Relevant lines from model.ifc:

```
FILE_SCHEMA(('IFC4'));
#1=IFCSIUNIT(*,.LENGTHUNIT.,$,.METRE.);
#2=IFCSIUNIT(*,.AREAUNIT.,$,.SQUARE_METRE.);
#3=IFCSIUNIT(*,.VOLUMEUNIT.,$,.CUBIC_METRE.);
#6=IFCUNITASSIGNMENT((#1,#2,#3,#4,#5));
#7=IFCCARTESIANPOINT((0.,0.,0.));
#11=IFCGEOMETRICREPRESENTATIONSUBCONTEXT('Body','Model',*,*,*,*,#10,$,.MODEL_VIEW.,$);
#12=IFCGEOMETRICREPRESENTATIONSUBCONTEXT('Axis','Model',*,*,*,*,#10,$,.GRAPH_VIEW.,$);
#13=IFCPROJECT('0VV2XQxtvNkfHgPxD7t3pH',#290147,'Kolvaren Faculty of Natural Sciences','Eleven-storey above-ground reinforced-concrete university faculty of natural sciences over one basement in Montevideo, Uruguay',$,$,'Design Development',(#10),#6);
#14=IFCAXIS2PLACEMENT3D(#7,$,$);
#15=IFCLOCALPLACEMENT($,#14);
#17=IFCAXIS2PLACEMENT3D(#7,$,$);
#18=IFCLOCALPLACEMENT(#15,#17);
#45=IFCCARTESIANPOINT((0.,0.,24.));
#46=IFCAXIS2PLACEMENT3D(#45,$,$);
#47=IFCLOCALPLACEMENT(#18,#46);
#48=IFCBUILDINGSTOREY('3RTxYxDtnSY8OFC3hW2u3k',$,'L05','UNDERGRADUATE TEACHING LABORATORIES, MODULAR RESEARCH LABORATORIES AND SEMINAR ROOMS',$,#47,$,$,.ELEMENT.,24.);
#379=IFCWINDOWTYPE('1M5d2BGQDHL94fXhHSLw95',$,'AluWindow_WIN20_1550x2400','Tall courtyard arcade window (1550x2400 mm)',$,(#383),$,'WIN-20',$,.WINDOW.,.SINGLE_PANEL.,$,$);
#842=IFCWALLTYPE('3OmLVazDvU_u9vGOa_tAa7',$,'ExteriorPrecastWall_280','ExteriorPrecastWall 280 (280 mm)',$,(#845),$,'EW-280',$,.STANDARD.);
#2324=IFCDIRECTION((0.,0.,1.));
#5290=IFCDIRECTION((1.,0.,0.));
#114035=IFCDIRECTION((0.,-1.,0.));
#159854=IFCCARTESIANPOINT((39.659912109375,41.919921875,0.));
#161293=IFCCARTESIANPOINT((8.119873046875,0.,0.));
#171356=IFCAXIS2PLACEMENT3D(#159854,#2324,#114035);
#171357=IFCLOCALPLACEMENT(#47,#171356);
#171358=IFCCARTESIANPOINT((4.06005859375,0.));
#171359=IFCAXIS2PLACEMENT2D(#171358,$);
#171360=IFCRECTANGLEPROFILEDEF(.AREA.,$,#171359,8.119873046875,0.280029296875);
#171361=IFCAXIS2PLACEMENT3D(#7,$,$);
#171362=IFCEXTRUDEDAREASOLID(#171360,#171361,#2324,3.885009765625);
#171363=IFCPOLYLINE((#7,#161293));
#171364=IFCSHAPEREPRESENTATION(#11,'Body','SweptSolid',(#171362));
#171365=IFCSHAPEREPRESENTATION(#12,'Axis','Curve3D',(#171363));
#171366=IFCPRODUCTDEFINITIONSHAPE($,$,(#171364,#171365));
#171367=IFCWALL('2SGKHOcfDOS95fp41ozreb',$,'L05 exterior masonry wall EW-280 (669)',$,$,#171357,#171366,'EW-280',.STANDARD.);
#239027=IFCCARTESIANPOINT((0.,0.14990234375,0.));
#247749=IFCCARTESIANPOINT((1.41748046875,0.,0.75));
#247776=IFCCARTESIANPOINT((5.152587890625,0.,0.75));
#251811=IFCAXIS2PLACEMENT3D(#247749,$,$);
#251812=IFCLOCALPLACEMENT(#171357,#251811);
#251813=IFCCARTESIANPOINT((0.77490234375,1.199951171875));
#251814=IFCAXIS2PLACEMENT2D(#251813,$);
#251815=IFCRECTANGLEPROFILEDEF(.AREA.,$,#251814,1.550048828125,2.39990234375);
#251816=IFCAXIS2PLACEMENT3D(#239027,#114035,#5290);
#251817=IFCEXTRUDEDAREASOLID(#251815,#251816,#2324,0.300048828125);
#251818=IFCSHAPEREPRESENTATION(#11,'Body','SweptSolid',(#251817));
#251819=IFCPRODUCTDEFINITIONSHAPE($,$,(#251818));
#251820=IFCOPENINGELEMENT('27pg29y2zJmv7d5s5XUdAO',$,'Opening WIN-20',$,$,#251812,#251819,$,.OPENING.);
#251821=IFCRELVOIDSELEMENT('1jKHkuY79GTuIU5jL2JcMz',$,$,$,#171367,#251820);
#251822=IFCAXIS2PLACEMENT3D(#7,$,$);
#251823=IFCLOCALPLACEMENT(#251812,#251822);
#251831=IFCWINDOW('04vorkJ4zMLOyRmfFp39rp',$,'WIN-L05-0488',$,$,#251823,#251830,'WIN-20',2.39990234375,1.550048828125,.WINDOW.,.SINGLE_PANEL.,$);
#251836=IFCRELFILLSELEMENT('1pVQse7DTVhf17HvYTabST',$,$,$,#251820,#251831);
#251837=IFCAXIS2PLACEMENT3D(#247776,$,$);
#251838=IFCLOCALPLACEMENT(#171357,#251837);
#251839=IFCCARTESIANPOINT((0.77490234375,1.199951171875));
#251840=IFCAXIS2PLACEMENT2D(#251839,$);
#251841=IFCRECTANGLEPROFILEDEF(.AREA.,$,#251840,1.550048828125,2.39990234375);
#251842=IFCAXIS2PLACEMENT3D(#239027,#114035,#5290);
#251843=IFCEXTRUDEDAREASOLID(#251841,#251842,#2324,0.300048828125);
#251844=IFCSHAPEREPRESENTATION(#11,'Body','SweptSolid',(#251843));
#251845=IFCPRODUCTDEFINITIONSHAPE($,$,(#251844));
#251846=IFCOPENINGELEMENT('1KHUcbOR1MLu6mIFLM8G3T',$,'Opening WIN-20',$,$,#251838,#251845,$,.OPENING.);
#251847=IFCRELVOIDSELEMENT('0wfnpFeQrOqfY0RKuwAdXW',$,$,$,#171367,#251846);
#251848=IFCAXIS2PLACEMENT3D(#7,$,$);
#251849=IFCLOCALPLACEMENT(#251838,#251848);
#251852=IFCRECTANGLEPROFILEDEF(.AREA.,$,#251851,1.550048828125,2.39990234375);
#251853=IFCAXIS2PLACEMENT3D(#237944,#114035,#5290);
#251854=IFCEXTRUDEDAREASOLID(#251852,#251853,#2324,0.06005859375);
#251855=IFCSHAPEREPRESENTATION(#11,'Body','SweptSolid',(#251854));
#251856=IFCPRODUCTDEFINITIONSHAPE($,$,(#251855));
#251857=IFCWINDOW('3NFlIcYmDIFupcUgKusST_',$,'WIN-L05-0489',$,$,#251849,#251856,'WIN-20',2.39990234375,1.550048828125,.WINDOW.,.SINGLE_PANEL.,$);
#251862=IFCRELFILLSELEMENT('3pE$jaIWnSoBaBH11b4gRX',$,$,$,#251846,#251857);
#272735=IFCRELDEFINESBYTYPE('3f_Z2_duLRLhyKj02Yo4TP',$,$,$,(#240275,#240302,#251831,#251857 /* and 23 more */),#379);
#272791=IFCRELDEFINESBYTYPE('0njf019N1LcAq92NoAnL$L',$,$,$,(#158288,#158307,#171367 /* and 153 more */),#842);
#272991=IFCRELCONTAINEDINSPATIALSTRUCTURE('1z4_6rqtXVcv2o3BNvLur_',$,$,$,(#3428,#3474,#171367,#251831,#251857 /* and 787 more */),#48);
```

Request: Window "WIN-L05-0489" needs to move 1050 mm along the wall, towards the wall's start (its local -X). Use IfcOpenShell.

```python
import ifcopenshell
import ifcopenshell.api.geometry
import ifcopenshell.util.placement

model = ifcopenshell.open("model.ifc")

window = model.by_guid("3NFlIcYmDIFupcUgKusST_")
opening = window.FillsVoids[0].RelatingOpeningElement
wall = opening.VoidsElements[0].RelatingBuildingElement

wall_matrix = ifcopenshell.util.placement.get_local_placement(wall.ObjectPlacement)
shift = wall_matrix[:3, 0] * -1.05
before = ifcopenshell.util.placement.get_local_placement(window.ObjectPlacement)[:3, 3].copy()

# The window is placed relative to its opening, so it follows when the opening moves.
matrix = ifcopenshell.util.placement.get_local_placement(opening.ObjectPlacement)
matrix[:3, 3] += shift
ifcopenshell.api.geometry.edit_object_placement(
    model, product=opening, matrix=matrix, is_si=False, should_transform_children=True
)

after = ifcopenshell.util.placement.get_local_placement(window.ObjectPlacement)[:3, 3]
print("window moved by", (after - before).round(3) + 0.0)

model.write("model_v2.ifc")
```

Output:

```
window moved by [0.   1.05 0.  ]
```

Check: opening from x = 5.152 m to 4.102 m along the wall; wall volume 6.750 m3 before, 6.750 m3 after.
